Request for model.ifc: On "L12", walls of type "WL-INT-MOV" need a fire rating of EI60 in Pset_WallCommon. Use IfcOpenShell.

First a look at what the model holds.

```python
import ifcopenshell
import ifcopenshell.util.element

model = ifcopenshell.open("model.ifc")
print(model.schema)
storey = next(s for s in model.by_type("IfcBuildingStorey") if s.Name == "L12")
walls = [e for e in ifcopenshell.util.element.get_decomposition(storey) if e.is_a("IfcWall")]
seen = {}
for e in walls:
    element_type = ifcopenshell.util.element.get_type(e)
    key = (element_type.Name if element_type != e and element_type else None, ifcopenshell.util.element.get_pset(e, "Pset_WallCommon", "FireRating"))
    seen[key] = seen.get(key, 0) + 1
for (name, value), count in sorted(seen.items(), key=str):
    print(count, "x", name, "|", value)
```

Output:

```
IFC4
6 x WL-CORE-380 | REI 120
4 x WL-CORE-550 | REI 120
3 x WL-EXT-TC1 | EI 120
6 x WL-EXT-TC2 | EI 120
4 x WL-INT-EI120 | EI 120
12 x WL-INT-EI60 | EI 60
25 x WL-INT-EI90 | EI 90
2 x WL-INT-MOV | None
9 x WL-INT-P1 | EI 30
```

```python
import ifcopenshell
import ifcopenshell.api.pset
import ifcopenshell.util.element

model = ifcopenshell.open("model.ifc")

storey = next(s for s in model.by_type("IfcBuildingStorey") if s.Name == "L12")
walls = [e for e in ifcopenshell.util.element.get_decomposition(storey) if e.is_a("IfcWall")]

count = 0
for e in walls:
    element_type = ifcopenshell.util.element.get_type(e)
    if element_type in (None, e) or element_type.Name != "WL-INT-MOV":
        continue
    found = ifcopenshell.util.element.get_pset(e, "Pset_WallCommon", should_inherit=False)
    if found:
        pset = model.by_id(found["id"])
        if len(ifcopenshell.util.element.get_elements_by_pset(pset)) > 1:
            pset = ifcopenshell.api.pset.unshare_pset(model, products=[e], pset=pset)[0]
    else:
        pset = ifcopenshell.api.pset.add_pset(model, product=e, name="Pset_WallCommon")
    ifcopenshell.api.pset.edit_pset(model, pset=pset, properties={"FireRating": "EI60"})
    count += 1

print(count, "walls updated")

model.write("model_rev.ifc")
```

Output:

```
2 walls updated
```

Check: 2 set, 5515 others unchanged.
